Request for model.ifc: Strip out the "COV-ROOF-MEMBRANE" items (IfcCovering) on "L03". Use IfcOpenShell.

First a look at what the model holds.

```python
import ifcopenshell
import ifcopenshell.util.element

model = ifcopenshell.open("model.ifc")
print(model.schema)
storey = next(s for s in model.by_type("IfcBuildingStorey") if s.Name == "L03")
coverings = [e for e in ifcopenshell.util.element.get_decomposition(storey) if e.is_a("IfcCovering")]
seen = {}
for e in coverings:
    element_type = ifcopenshell.util.element.get_type(e)
    name = element_type.Name if element_type not in (None, e) else None
    seen[name] = seen.get(name, 0) + 1
for name, count in sorted(seen.items(), key=str):
    print(count, "x", name)
```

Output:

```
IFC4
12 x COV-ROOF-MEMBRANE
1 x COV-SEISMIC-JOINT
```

```python
import ifcopenshell
import ifcopenshell.api.root
import ifcopenshell.util.element

model = ifcopenshell.open("model.ifc")

storey = next(s for s in model.by_type("IfcBuildingStorey") if s.Name == "L03")
coverings = [e for e in ifcopenshell.util.element.get_decomposition(storey) if e.is_a("IfcCovering")]
targets = [e for e in coverings if (t := ifcopenshell.util.element.get_type(e)) not in (None, e) and t.Name == "COV-ROOF-MEMBRANE"]

for e in targets:
    ifcopenshell.api.root.remove_product(model, product=e)
print(len(targets), "removed")

model.write("model_edited.ifc")
```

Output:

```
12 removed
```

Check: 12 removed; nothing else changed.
